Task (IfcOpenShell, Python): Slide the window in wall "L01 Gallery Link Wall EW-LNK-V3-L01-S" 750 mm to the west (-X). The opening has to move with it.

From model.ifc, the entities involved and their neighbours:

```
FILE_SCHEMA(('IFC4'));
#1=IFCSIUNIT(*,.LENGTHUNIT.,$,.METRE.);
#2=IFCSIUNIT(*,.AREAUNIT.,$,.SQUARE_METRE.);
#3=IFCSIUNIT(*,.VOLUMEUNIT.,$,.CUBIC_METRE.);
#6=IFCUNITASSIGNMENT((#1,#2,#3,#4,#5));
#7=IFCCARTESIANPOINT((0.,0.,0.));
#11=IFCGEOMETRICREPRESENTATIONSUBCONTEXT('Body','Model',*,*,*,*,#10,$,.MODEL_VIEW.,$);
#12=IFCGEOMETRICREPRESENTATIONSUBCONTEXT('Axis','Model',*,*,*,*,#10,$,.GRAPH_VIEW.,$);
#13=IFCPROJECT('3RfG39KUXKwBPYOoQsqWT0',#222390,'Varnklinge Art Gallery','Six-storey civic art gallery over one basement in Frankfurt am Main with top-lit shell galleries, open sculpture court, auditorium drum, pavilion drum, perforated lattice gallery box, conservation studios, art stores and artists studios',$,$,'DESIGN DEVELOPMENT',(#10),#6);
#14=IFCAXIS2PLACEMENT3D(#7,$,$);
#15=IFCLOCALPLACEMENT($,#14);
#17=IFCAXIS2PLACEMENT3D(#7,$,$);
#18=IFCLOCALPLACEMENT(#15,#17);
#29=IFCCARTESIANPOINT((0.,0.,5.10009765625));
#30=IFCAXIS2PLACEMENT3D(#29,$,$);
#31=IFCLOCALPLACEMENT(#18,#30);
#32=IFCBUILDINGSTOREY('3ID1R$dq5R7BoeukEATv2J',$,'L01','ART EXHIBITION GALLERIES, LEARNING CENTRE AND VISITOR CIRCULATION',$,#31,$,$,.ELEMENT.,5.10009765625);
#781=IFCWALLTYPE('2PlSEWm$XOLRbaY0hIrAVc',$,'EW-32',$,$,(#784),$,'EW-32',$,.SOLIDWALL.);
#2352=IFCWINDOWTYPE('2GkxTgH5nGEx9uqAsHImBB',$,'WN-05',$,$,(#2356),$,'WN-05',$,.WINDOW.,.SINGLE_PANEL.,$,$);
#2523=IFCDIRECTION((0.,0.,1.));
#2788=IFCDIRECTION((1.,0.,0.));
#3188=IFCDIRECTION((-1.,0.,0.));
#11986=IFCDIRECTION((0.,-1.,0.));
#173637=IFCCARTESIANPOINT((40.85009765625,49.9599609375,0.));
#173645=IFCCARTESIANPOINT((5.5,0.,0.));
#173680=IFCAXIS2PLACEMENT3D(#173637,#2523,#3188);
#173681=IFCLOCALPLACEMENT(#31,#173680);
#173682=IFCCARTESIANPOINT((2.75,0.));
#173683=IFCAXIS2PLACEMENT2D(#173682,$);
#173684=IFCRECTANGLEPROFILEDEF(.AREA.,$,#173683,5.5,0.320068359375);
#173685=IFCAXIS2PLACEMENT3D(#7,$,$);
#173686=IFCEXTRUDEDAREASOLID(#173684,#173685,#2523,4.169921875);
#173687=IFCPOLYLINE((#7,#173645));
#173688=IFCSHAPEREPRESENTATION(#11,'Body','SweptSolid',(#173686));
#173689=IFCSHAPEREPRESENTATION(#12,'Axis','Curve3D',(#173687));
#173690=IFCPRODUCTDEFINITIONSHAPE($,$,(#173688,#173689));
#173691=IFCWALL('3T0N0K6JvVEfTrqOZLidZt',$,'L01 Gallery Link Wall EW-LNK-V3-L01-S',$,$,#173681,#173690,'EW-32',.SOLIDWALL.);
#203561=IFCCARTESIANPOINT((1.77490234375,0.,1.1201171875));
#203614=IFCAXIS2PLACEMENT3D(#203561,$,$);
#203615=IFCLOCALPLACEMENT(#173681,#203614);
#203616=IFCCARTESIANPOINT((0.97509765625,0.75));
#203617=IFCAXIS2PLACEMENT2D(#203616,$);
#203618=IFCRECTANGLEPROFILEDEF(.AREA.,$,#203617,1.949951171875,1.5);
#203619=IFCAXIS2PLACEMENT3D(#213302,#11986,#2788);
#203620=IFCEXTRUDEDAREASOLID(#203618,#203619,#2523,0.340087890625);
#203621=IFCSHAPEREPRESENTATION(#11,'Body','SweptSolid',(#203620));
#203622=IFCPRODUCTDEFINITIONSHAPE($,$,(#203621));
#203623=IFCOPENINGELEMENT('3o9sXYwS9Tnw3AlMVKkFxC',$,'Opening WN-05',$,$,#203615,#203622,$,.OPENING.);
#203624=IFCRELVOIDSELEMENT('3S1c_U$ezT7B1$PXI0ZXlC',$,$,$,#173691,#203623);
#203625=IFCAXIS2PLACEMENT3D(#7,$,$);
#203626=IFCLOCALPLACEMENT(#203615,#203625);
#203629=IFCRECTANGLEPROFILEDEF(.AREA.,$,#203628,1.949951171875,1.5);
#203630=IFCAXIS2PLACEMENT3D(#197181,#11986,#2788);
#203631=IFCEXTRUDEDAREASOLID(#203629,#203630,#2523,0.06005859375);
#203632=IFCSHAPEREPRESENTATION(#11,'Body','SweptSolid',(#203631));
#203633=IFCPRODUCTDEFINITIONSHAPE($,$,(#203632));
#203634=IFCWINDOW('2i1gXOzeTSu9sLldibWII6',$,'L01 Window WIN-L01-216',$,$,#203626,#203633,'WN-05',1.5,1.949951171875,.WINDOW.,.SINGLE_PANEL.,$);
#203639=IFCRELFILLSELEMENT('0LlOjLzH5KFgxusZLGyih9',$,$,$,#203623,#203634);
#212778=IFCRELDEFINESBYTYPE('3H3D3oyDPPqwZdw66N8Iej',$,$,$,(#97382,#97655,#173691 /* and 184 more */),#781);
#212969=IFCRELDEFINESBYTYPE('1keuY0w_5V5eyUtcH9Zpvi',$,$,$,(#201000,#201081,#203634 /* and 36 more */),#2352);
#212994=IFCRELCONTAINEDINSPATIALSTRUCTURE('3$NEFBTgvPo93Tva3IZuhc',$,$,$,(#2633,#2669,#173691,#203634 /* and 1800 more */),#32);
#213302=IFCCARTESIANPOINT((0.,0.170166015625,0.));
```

```python
import ifcopenshell
import ifcopenshell.api.geometry
import ifcopenshell.util.placement
import ifcopenshell.util.unit

model = ifcopenshell.open("model.ifc")
unit_scale = ifcopenshell.util.unit.calculate_unit_scale(model)

window = model.by_guid("2i1gXOzeTSu9sLldibWII6")
opening = window.FillsVoids[0].RelatingOpeningElement
wall = opening.VoidsElements[0].RelatingBuildingElement

wall_matrix = ifcopenshell.util.placement.get_local_placement(wall.ObjectPlacement)
shift = wall_matrix[:3, 0] * 0.75 / unit_scale
before = ifcopenshell.util.placement.get_local_placement(window.ObjectPlacement)[:3, 3].copy()

# The window is placed relative to its opening, so it follows when the opening moves.
matrix = ifcopenshell.util.placement.get_local_placement(opening.ObjectPlacement)
matrix[:3, 3] += shift
ifcopenshell.api.geometry.edit_object_placement(
    model, product=opening, matrix=matrix, is_si=False, should_transform_children=True
)

after = ifcopenshell.util.placement.get_local_placement(window.ObjectPlacement)[:3, 3]
print("window moved by", (after - before).round(3) + 0.0)

model.write("model_updated.ifc")
```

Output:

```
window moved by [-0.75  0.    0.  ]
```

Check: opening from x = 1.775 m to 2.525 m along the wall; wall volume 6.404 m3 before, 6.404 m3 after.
